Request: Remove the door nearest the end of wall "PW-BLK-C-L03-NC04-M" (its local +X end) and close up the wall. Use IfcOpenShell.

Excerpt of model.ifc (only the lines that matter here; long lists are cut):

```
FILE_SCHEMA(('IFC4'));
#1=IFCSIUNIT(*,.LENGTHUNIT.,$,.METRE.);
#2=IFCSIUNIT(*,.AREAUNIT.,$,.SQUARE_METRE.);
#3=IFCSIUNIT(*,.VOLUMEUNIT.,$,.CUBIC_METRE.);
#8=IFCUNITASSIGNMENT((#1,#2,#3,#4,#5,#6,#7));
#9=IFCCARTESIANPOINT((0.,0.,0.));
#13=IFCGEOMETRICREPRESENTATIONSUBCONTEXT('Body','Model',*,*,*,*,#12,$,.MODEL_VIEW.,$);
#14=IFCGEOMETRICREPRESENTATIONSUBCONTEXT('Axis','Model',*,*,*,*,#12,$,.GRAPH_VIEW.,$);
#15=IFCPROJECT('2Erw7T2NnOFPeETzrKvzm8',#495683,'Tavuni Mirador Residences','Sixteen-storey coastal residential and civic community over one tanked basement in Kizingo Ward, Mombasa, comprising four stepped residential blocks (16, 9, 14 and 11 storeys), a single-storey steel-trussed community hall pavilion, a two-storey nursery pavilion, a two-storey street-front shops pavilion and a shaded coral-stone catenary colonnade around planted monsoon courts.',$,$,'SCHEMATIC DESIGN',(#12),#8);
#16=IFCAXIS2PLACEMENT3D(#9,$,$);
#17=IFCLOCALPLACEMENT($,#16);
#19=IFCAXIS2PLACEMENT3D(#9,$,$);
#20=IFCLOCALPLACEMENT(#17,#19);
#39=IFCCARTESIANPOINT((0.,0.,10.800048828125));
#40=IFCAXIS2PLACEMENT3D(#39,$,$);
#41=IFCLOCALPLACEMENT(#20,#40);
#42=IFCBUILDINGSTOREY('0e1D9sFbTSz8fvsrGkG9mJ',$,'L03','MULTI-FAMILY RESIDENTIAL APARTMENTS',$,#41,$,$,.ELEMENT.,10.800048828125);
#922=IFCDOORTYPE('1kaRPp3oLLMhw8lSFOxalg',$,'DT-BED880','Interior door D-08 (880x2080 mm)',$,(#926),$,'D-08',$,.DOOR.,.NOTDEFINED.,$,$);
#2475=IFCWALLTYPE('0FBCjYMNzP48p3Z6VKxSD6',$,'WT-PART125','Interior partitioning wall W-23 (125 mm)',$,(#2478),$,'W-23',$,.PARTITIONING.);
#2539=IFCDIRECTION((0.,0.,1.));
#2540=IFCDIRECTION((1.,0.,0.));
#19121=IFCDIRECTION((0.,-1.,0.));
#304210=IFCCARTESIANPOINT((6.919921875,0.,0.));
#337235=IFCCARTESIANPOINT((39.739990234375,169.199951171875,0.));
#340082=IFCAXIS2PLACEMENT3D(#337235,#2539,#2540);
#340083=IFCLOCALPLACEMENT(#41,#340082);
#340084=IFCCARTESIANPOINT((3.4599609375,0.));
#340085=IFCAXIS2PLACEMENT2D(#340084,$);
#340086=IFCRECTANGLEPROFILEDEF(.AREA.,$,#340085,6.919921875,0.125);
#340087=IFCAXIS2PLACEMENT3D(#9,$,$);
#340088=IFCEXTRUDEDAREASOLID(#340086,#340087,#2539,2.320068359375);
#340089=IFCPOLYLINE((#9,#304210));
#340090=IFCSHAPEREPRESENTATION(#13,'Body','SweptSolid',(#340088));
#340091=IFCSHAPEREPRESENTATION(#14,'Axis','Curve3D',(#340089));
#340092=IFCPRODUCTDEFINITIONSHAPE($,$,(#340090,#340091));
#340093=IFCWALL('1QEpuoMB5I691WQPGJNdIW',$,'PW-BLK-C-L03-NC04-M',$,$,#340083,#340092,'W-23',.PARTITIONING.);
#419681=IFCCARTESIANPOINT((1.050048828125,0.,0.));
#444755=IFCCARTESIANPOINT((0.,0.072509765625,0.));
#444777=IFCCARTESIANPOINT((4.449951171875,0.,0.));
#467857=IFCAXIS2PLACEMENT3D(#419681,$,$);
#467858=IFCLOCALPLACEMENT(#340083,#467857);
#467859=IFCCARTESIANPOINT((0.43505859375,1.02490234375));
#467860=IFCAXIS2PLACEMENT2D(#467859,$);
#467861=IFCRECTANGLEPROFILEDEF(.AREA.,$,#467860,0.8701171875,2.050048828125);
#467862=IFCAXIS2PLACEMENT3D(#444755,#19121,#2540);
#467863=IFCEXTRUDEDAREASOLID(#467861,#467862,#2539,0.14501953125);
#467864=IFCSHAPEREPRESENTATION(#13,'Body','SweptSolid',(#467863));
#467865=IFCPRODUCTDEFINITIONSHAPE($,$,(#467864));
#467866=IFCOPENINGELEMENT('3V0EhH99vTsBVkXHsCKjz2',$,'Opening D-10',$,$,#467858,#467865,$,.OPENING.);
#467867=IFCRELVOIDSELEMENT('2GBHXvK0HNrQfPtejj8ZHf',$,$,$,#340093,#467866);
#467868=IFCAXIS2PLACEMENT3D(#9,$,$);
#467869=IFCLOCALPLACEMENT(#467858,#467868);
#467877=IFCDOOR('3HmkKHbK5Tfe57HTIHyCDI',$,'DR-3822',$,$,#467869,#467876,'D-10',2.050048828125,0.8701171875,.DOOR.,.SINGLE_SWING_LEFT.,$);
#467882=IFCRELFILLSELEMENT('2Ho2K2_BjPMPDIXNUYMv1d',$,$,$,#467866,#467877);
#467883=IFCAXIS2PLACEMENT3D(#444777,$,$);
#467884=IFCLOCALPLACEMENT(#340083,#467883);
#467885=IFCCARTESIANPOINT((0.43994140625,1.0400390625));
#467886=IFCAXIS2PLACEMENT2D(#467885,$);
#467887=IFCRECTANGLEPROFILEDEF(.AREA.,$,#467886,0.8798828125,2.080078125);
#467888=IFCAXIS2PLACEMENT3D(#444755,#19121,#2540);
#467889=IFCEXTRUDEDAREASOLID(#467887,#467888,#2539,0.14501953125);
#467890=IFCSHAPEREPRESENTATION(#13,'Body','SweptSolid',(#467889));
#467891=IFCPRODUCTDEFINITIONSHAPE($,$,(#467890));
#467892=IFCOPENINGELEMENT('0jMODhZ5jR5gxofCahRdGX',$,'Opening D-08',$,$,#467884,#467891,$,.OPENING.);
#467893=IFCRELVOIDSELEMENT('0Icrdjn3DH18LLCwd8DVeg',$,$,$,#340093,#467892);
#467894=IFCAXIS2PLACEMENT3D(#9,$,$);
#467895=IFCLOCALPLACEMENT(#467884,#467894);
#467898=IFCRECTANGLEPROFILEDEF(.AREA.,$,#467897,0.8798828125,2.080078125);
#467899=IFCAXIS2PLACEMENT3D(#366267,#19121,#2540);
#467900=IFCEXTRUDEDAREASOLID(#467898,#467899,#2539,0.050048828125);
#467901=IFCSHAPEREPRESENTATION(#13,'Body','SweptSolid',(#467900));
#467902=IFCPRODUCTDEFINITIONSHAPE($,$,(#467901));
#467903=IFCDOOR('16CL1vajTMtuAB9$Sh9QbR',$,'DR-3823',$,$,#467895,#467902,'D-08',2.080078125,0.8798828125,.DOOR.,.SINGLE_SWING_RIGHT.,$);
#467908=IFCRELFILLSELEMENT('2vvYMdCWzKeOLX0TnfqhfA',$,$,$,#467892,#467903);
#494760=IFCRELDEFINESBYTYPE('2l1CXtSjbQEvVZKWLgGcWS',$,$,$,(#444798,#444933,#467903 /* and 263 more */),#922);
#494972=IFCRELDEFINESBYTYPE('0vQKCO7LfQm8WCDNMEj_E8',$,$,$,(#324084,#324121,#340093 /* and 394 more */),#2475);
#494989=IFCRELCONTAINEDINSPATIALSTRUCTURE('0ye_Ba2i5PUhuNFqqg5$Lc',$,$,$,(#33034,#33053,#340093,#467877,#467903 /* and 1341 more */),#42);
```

```python
import ifcopenshell
import ifcopenshell.api.feature
import ifcopenshell.api.root
import ifcopenshell.geom
import ifcopenshell.util.shape

model = ifcopenshell.open("model.ifc")
settings = ifcopenshell.geom.settings()


def volume(element):
    """Net volume in cubic metres, openings subtracted."""
    shape = ifcopenshell.geom.create_shape(settings, element)
    return ifcopenshell.util.shape.get_volume(shape.geometry)


door = model.by_guid("16CL1vajTMtuAB9$Sh9QbR")
opening = door.FillsVoids[0].RelatingOpeningElement
wall = opening.VoidsElements[0].RelatingBuildingElement
before = volume(wall)

ifcopenshell.api.root.remove_product(model, product=door)
ifcopenshell.api.feature.remove_feature(model, feature=opening)

after = volume(wall)

print(f"wall volume {before:.3f} -> {after:.3f} m3")

model.write("model_updated.ifc")
```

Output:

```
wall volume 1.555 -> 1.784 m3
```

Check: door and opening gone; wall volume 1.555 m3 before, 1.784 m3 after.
